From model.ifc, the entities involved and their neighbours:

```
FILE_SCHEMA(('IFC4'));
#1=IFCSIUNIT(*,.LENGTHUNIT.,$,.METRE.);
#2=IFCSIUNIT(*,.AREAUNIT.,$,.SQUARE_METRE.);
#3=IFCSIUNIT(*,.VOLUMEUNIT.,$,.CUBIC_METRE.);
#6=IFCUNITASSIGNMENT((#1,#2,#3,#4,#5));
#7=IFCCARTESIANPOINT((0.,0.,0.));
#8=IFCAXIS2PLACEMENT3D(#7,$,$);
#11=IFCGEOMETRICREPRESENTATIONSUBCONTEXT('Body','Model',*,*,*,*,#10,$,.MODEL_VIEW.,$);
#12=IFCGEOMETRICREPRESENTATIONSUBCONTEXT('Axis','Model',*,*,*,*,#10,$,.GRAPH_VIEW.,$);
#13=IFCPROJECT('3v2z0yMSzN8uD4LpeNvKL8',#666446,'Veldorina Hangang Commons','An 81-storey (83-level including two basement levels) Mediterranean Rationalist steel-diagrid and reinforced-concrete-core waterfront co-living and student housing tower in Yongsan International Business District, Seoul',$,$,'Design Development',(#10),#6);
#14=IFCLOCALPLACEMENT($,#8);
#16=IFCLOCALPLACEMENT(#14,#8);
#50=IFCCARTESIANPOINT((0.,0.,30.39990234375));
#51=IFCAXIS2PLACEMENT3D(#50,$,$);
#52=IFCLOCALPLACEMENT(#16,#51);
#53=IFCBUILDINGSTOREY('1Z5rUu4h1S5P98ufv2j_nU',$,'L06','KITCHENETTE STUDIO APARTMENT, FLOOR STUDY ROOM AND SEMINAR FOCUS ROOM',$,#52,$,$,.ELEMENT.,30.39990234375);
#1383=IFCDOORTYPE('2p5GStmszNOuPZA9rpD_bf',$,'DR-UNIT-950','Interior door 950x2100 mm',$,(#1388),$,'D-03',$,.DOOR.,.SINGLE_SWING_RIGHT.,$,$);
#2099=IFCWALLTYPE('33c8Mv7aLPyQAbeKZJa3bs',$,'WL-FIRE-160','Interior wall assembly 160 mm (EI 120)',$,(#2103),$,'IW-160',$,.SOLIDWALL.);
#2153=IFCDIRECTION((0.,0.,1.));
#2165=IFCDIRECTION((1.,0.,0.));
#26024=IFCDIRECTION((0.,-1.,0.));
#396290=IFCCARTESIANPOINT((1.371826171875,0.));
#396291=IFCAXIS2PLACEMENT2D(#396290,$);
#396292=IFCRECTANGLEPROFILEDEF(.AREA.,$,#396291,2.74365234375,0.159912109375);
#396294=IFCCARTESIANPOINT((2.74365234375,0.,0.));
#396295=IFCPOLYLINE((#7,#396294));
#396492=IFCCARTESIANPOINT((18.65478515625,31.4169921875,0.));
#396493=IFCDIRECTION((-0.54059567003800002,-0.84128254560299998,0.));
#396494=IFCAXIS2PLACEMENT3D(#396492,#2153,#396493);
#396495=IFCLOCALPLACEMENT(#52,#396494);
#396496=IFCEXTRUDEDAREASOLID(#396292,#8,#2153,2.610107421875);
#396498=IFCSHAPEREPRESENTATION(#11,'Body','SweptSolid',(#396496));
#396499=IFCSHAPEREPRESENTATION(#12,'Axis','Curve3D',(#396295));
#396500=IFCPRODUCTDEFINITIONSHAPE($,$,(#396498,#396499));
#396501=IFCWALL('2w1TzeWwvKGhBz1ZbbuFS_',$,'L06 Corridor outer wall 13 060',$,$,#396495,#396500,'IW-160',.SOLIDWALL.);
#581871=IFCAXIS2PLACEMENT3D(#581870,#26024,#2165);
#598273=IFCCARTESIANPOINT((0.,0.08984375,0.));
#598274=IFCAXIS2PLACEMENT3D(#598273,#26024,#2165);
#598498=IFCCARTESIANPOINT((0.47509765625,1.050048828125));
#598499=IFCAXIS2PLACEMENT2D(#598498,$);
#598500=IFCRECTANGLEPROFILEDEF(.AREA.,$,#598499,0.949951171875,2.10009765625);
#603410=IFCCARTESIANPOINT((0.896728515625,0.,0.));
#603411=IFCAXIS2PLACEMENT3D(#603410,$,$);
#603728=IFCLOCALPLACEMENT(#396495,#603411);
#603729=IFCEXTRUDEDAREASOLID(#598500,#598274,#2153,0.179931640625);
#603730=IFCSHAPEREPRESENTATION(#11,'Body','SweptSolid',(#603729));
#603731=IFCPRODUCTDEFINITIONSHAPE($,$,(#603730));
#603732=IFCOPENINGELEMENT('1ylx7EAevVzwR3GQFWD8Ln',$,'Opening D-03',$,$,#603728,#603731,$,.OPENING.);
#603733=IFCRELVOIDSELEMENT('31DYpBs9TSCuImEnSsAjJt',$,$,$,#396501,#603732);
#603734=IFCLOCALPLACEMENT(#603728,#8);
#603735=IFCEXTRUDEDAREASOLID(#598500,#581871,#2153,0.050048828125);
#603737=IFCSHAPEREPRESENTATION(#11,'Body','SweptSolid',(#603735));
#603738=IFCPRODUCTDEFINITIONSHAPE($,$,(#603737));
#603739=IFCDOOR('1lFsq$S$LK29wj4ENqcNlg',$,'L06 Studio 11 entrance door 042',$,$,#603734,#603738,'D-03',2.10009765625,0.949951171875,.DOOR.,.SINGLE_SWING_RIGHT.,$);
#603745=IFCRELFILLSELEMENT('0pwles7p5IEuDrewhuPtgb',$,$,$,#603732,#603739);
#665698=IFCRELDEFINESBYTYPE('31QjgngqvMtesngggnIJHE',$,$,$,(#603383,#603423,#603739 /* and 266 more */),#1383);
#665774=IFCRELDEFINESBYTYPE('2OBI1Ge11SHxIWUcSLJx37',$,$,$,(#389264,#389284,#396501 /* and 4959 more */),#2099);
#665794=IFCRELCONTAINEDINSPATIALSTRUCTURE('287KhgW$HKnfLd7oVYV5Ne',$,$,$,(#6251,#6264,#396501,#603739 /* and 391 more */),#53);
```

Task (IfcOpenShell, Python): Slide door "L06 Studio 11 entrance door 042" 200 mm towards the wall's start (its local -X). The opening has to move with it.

```python
import ifcopenshell
import ifcopenshell.api.geometry
import ifcopenshell.util.placement
import ifcopenshell.util.unit

model = ifcopenshell.open("model.ifc")
unit_scale = ifcopenshell.util.unit.calculate_unit_scale(model)

door = model.by_guid("1lFsq$S$LK29wj4ENqcNlg")
opening = door.FillsVoids[0].RelatingOpeningElement
wall = opening.VoidsElements[0].RelatingBuildingElement

wall_matrix = ifcopenshell.util.placement.get_local_placement(wall.ObjectPlacement)
shift = wall_matrix[:3, 0] * -0.2 / unit_scale
before = ifcopenshell.util.placement.get_local_placement(door.ObjectPlacement)[:3, 3].copy()

# The door is placed relative to its opening, so it follows when the opening moves.
matrix = ifcopenshell.util.placement.get_local_placement(opening.ObjectPlacement)
matrix[:3, 3] += shift
ifcopenshell.api.geometry.edit_object_placement(
    model, product=opening, matrix=matrix, is_si=False, should_transform_children=True
)

after = ifcopenshell.util.placement.get_local_placement(door.ObjectPlacement)[:3, 3]
print("door moved by", (after - before).round(3) + 0.0)

model.write("model-out.ifc")
```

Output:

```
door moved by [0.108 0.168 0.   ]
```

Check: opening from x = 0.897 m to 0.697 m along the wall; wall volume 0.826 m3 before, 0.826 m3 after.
